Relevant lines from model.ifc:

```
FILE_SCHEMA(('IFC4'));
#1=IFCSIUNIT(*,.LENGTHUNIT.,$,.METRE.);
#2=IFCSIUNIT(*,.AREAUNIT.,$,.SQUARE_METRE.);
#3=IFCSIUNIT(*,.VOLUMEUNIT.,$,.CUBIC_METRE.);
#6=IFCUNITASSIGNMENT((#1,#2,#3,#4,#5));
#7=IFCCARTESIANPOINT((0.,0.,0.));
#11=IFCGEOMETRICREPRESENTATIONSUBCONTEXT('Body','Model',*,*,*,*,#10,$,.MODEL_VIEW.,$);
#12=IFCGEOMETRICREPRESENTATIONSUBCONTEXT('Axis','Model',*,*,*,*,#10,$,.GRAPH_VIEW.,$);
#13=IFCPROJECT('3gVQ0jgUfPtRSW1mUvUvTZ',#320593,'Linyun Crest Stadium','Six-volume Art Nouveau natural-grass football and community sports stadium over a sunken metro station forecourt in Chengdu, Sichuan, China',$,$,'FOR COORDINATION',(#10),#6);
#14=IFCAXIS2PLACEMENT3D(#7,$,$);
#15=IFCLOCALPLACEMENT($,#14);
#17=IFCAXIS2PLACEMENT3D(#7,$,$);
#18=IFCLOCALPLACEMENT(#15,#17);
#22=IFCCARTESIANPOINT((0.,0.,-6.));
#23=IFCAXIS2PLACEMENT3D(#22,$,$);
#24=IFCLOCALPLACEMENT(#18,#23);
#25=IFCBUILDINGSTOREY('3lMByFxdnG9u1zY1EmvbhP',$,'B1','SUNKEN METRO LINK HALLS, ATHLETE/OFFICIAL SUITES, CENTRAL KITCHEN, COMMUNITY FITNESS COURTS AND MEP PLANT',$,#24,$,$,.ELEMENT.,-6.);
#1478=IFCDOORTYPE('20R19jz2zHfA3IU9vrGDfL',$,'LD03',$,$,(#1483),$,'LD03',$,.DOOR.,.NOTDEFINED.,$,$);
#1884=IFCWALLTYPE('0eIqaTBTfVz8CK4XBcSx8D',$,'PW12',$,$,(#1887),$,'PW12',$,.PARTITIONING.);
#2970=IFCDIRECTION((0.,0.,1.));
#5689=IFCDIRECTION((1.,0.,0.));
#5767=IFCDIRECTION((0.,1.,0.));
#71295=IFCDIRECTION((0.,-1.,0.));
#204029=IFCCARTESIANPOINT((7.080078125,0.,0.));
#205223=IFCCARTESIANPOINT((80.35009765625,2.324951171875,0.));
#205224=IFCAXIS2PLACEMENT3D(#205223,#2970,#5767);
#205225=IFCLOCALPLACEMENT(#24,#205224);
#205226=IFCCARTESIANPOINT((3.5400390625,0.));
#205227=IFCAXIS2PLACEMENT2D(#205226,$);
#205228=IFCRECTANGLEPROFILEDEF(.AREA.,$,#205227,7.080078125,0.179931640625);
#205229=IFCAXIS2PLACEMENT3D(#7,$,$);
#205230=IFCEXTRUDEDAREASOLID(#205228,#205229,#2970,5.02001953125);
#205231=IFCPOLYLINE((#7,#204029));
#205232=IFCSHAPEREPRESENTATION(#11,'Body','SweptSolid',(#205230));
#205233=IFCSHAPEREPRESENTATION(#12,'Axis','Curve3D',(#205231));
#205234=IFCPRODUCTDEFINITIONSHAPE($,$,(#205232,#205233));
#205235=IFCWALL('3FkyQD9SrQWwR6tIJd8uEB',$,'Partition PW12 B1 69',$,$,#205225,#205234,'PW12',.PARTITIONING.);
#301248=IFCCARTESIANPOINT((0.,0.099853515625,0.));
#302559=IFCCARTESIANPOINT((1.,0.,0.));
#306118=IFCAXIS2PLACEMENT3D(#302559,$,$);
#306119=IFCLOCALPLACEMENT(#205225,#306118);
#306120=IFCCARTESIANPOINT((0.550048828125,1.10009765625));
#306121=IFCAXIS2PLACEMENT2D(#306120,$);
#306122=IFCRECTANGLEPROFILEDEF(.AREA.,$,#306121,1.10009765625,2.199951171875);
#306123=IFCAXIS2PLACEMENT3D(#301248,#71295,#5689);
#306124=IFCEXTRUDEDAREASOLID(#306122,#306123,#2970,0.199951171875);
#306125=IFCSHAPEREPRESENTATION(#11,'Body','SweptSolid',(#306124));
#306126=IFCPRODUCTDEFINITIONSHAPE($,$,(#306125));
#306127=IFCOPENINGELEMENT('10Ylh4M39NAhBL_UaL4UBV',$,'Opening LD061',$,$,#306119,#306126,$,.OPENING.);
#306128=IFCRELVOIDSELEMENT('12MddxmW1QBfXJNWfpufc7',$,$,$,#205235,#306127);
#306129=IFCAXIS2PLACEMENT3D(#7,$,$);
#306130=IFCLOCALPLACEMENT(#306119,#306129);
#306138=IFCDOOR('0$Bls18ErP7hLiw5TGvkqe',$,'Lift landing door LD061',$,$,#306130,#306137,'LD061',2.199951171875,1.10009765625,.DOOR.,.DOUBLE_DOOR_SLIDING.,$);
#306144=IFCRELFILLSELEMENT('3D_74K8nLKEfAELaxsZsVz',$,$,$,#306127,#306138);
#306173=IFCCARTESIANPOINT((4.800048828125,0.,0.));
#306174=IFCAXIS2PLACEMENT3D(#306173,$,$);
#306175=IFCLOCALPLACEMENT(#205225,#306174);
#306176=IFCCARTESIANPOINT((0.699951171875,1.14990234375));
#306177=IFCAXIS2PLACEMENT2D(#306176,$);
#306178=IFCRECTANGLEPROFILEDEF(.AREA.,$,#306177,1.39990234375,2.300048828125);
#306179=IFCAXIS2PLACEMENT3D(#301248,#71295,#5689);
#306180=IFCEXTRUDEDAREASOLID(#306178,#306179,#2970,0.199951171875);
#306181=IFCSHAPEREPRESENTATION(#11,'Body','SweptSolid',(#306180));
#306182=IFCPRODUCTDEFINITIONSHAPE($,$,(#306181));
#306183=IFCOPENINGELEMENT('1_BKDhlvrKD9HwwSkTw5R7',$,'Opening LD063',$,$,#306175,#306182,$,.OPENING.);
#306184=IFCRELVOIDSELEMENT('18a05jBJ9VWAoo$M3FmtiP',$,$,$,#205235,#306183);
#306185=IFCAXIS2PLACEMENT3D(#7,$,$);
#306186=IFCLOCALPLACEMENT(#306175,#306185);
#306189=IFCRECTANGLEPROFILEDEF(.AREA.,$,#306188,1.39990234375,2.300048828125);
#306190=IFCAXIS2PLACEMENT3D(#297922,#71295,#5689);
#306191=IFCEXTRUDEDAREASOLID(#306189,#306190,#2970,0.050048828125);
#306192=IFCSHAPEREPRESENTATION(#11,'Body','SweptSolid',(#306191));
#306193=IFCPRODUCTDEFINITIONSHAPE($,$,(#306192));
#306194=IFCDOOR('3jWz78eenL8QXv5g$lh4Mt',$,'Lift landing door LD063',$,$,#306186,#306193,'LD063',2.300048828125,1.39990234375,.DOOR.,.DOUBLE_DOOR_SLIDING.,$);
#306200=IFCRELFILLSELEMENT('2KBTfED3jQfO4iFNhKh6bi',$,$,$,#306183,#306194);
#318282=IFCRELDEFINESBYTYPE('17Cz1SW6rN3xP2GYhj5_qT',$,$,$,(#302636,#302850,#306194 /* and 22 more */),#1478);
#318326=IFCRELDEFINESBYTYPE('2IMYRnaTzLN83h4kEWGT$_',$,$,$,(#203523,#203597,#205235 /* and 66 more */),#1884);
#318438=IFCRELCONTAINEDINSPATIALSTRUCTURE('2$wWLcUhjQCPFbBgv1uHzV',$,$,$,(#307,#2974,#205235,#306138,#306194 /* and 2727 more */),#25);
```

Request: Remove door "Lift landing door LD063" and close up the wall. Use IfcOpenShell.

```python
import ifcopenshell
import ifcopenshell.api.feature
import ifcopenshell.api.root
import ifcopenshell.geom
import ifcopenshell.util.shape

model = ifcopenshell.open("model.ifc")
settings = ifcopenshell.geom.settings()


def volume(element):
    """Net volume in cubic metres, openings subtracted."""
    shape = ifcopenshell.geom.create_shape(settings, element)
    return ifcopenshell.util.shape.get_volume(shape.geometry)


door = model.by_guid("3jWz78eenL8QXv5g$lh4Mt")
opening = door.FillsVoids[0].RelatingOpeningElement
wall = opening.VoidsElements[0].RelatingBuildingElement
before = volume(wall)

ifcopenshell.api.root.remove_product(model, product=door)
ifcopenshell.api.feature.remove_feature(model, feature=opening)

after = volume(wall)

print(f"wall volume {before:.3f} -> {after:.3f} m3")

model.write("model_rev.ifc")
```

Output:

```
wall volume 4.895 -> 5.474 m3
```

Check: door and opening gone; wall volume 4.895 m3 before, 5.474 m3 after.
